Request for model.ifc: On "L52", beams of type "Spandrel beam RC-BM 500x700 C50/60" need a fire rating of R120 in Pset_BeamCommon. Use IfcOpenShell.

First a look at what the model holds.

```python
import ifcopenshell
import ifcopenshell.util.element

model = ifcopenshell.open("model.ifc")
print(model.schema)
storey = next(s for s in model.by_type("IfcBuildingStorey") if s.Name == "L52")
beams = [e for e in ifcopenshell.util.element.get_decomposition(storey) if e.is_a("IfcBeam")]
seen = {}
for e in beams:
    element_type = ifcopenshell.util.element.get_type(e)
    key = (element_type.Name if element_type != e and element_type else None, ifcopenshell.util.element.get_pset(e, "Pset_BeamCommon", "FireRating"))
    seen[key] = seen.get(key, 0) + 1
for (name, value), count in sorted(seen.items(), key=str):
    print(count, "x", name, "|", value)
```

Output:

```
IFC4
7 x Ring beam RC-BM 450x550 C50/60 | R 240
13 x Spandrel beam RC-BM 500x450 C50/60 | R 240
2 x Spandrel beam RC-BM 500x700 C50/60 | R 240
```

```python
import ifcopenshell
import ifcopenshell.api.pset
import ifcopenshell.util.element

model = ifcopenshell.open("model.ifc")

storey = next(s for s in model.by_type("IfcBuildingStorey") if s.Name == "L52")
beams = [e for e in ifcopenshell.util.element.get_decomposition(storey) if e.is_a("IfcBeam")]

count = 0
for e in beams:
    element_type = ifcopenshell.util.element.get_type(e)
    if element_type in (None, e) or element_type.Name != "Spandrel beam RC-BM 500x700 C50/60":
        continue
    found = ifcopenshell.util.element.get_pset(e, "Pset_BeamCommon", should_inherit=False)
    if found:
        pset = model.by_id(found["id"])
        if len(ifcopenshell.util.element.get_elements_by_pset(pset)) > 1:
            pset = ifcopenshell.api.pset.unshare_pset(model, products=[e], pset=pset)[0]
    else:
        pset = ifcopenshell.api.pset.add_pset(model, product=e, name="Pset_BeamCommon")
    ifcopenshell.api.pset.edit_pset(model, pset=pset, properties={"FireRating": "R120"})
    count += 1

print(count, "beams updated")

model.write("model_edited.ifc")
```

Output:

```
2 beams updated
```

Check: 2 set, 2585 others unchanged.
